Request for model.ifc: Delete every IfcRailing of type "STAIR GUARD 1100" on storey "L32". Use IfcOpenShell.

First a look at what the model holds.

```python
import ifcopenshell
import ifcopenshell.util.element

model = ifcopenshell.open("model.ifc")
print(model.schema)
storey = next(s for s in model.by_type("IfcBuildingStorey") if s.Name == "L32")
railings = [e for e in ifcopenshell.util.element.get_decomposition(storey) if e.is_a("IfcRailing")]
seen = {}
for e in railings:
    element_type = ifcopenshell.util.element.get_type(e)
    name = element_type.Name if element_type not in (None, e) else None
    seen[name] = seen.get(name, 0) + 1
for name, count in sorted(seen.items(), key=str):
    print(count, "x", name)
```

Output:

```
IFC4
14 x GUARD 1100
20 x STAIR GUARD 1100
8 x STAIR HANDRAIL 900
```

```python
import ifcopenshell
import ifcopenshell.api.root
import ifcopenshell.util.element

model = ifcopenshell.open("model.ifc")

storey = next(s for s in model.by_type("IfcBuildingStorey") if s.Name == "L32")
railings = [e for e in ifcopenshell.util.element.get_decomposition(storey) if e.is_a("IfcRailing")]
targets = [e for e in railings if (t := ifcopenshell.util.element.get_type(e)) not in (None, e) and t.Name == "STAIR GUARD 1100"]

for e in targets:
    ifcopenshell.api.root.remove_product(model, product=e)
print(len(targets), "removed")

model.write("model_v2.ifc")
```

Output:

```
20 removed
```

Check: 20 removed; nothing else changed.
